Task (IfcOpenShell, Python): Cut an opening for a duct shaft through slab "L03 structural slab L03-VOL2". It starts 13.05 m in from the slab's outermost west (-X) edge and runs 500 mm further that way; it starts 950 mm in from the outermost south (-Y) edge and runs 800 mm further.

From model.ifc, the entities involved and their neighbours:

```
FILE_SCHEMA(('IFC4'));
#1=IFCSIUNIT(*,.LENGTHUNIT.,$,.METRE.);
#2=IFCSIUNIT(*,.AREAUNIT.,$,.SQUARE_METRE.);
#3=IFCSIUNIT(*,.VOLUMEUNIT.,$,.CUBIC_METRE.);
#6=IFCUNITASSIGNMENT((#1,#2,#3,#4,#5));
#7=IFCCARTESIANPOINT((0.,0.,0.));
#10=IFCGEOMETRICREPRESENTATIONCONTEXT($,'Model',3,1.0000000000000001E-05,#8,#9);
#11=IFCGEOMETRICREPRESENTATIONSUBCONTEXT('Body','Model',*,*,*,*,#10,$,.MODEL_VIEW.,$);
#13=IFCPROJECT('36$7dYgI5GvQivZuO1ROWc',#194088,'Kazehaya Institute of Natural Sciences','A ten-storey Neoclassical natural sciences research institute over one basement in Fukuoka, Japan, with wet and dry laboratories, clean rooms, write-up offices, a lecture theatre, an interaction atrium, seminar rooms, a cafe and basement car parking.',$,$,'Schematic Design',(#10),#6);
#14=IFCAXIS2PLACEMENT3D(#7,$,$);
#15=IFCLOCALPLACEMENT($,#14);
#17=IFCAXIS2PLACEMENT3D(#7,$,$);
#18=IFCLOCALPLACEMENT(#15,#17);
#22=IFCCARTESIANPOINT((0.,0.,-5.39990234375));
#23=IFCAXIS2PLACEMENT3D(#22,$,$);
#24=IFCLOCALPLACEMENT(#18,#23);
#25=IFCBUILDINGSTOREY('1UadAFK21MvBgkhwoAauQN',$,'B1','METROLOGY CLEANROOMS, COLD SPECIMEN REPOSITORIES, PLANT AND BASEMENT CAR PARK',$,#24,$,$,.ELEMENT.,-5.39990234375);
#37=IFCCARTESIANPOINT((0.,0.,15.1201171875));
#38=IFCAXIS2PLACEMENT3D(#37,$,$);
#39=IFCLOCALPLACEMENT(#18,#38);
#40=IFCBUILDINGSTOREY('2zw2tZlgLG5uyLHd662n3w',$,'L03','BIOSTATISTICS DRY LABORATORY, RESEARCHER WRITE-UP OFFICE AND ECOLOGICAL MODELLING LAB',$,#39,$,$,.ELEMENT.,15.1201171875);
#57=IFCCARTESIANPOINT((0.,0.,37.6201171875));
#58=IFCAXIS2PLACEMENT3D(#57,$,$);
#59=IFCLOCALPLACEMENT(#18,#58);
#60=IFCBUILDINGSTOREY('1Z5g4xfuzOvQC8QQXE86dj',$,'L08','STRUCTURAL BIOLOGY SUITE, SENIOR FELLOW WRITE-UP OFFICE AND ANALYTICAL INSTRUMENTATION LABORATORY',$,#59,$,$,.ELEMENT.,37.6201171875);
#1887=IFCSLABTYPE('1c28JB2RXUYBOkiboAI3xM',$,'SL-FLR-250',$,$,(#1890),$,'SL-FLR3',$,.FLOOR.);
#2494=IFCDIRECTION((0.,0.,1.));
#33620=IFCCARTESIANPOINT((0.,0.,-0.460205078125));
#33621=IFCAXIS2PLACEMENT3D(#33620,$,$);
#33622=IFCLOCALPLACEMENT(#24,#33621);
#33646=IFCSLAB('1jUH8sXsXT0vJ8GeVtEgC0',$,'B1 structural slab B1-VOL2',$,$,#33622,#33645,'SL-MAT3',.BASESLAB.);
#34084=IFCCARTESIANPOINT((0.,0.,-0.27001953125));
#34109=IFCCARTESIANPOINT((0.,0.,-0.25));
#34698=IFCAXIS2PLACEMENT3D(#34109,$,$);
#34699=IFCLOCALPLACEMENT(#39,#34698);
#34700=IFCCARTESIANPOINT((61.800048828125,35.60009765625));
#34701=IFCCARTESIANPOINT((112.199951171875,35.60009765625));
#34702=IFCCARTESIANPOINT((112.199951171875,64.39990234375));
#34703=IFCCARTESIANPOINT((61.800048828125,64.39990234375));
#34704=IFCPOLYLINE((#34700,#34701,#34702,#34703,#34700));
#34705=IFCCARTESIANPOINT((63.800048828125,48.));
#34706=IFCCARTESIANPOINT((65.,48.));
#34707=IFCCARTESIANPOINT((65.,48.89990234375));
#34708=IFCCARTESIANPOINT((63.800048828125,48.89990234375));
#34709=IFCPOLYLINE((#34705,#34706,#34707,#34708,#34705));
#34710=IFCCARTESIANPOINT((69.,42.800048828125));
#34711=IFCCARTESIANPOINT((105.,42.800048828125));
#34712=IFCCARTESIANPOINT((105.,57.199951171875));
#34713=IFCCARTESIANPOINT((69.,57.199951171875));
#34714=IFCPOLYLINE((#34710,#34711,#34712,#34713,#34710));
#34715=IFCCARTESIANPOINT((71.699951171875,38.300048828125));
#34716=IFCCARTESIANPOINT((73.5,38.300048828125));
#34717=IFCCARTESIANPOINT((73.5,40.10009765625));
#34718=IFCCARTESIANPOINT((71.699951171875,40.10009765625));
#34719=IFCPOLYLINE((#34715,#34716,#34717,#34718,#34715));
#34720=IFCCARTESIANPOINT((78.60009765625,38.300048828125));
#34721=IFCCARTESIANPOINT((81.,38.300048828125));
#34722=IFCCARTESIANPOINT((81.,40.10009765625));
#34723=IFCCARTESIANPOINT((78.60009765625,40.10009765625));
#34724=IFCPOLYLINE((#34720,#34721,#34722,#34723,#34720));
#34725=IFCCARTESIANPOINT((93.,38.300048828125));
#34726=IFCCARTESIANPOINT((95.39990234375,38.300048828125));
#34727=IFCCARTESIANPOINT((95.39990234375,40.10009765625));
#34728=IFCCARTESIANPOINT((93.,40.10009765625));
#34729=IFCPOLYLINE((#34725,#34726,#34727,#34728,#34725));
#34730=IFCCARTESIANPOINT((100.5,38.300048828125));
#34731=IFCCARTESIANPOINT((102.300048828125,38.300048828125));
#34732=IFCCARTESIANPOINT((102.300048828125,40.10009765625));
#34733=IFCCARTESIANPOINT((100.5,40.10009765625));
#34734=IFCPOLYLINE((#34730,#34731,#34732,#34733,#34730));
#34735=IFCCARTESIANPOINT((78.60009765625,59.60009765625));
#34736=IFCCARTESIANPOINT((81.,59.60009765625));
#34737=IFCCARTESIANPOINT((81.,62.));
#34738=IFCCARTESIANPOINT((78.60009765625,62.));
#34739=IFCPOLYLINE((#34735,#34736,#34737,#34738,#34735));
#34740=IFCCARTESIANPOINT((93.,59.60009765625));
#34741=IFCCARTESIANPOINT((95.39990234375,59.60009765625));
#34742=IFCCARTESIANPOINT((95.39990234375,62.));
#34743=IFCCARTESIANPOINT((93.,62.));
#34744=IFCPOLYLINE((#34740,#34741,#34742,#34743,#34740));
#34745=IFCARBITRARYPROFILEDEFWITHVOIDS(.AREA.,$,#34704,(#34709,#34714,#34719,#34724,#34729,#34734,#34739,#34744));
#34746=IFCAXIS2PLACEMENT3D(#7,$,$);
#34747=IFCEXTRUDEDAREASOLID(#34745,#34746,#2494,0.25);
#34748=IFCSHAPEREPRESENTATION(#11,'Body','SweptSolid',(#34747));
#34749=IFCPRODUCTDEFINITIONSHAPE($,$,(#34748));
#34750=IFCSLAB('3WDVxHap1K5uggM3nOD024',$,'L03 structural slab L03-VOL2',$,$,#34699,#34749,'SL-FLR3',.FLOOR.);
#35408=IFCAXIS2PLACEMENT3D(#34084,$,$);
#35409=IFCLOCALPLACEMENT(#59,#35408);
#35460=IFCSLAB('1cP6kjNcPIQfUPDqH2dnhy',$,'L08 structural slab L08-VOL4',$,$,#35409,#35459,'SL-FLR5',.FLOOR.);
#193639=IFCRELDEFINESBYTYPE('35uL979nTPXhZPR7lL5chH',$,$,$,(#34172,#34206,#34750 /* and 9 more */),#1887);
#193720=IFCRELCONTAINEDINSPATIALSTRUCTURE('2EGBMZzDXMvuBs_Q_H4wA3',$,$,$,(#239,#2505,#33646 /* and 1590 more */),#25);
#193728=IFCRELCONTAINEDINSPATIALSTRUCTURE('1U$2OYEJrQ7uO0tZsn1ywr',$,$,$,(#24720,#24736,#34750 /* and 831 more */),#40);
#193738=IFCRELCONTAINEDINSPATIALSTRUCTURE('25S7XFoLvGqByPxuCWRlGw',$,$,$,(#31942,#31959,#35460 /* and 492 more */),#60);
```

```python
import numpy as np
import ifcopenshell
import ifcopenshell.api.feature
import ifcopenshell.api.geometry
import ifcopenshell.api.root
import ifcopenshell.geom
import ifcopenshell.util.placement
import ifcopenshell.util.representation
import ifcopenshell.util.shape
import ifcopenshell.util.unit

model = ifcopenshell.open("model.ifc")
unit_scale = ifcopenshell.util.unit.calculate_unit_scale(model)
settings = ifcopenshell.geom.settings()


def volume(element):
    """Net volume in cubic metres, openings subtracted."""
    shape = ifcopenshell.geom.create_shape(settings, element)
    return ifcopenshell.util.shape.get_volume(shape.geometry)


slab = model.by_id(34750)
before = volume(slab)

# Extent in the slab's own axes, in metres. The edges named are its -X and -Y sides.
slab_shape = ifcopenshell.geom.create_shape(settings, slab)
vertices = ifcopenshell.util.shape.get_vertices(slab_shape.geometry)
x_min, y_min, bottom = vertices.min(axis=0)
top = vertices[:, 2].max()

opening = ifcopenshell.api.root.create_entity(model, ifc_class="IfcOpeningElement", name="Duct shaft opening", predefined_type="OPENING")
context = ifcopenshell.util.representation.get_context(model, "Model", "Body", "MODEL_VIEW")
width, depth = 0.5, 0.8
outline = [(0.0, 0.0), (width, 0.0), (width, depth), (0.0, depth), (0.0, 0.0)]
# Overshoot both faces by 50 mm so the cut is clean.
shape = ifcopenshell.api.geometry.add_slab_representation(
    model, context=context, depth=top - bottom + 0.1, polyline=outline
)
ifcopenshell.api.geometry.assign_representation(model, product=opening, representation=shape)

matrix = ifcopenshell.util.placement.get_local_placement(slab.ObjectPlacement)
matrix[:, 3] = matrix @ np.append(np.array([x_min + 13.05, y_min + 0.95, bottom - 0.05]) / unit_scale, 1.0)
ifcopenshell.api.geometry.edit_object_placement(model, product=opening, matrix=matrix, is_si=False)
ifcopenshell.api.feature.add_feature(model, feature=opening, element=slab)

after = volume(slab)

print(f"slab volume {before:.3f} -> {after:.3f} m3")

model.write("model_v2.ifc")
```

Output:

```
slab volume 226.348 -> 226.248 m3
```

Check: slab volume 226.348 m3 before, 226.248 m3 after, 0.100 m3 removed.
